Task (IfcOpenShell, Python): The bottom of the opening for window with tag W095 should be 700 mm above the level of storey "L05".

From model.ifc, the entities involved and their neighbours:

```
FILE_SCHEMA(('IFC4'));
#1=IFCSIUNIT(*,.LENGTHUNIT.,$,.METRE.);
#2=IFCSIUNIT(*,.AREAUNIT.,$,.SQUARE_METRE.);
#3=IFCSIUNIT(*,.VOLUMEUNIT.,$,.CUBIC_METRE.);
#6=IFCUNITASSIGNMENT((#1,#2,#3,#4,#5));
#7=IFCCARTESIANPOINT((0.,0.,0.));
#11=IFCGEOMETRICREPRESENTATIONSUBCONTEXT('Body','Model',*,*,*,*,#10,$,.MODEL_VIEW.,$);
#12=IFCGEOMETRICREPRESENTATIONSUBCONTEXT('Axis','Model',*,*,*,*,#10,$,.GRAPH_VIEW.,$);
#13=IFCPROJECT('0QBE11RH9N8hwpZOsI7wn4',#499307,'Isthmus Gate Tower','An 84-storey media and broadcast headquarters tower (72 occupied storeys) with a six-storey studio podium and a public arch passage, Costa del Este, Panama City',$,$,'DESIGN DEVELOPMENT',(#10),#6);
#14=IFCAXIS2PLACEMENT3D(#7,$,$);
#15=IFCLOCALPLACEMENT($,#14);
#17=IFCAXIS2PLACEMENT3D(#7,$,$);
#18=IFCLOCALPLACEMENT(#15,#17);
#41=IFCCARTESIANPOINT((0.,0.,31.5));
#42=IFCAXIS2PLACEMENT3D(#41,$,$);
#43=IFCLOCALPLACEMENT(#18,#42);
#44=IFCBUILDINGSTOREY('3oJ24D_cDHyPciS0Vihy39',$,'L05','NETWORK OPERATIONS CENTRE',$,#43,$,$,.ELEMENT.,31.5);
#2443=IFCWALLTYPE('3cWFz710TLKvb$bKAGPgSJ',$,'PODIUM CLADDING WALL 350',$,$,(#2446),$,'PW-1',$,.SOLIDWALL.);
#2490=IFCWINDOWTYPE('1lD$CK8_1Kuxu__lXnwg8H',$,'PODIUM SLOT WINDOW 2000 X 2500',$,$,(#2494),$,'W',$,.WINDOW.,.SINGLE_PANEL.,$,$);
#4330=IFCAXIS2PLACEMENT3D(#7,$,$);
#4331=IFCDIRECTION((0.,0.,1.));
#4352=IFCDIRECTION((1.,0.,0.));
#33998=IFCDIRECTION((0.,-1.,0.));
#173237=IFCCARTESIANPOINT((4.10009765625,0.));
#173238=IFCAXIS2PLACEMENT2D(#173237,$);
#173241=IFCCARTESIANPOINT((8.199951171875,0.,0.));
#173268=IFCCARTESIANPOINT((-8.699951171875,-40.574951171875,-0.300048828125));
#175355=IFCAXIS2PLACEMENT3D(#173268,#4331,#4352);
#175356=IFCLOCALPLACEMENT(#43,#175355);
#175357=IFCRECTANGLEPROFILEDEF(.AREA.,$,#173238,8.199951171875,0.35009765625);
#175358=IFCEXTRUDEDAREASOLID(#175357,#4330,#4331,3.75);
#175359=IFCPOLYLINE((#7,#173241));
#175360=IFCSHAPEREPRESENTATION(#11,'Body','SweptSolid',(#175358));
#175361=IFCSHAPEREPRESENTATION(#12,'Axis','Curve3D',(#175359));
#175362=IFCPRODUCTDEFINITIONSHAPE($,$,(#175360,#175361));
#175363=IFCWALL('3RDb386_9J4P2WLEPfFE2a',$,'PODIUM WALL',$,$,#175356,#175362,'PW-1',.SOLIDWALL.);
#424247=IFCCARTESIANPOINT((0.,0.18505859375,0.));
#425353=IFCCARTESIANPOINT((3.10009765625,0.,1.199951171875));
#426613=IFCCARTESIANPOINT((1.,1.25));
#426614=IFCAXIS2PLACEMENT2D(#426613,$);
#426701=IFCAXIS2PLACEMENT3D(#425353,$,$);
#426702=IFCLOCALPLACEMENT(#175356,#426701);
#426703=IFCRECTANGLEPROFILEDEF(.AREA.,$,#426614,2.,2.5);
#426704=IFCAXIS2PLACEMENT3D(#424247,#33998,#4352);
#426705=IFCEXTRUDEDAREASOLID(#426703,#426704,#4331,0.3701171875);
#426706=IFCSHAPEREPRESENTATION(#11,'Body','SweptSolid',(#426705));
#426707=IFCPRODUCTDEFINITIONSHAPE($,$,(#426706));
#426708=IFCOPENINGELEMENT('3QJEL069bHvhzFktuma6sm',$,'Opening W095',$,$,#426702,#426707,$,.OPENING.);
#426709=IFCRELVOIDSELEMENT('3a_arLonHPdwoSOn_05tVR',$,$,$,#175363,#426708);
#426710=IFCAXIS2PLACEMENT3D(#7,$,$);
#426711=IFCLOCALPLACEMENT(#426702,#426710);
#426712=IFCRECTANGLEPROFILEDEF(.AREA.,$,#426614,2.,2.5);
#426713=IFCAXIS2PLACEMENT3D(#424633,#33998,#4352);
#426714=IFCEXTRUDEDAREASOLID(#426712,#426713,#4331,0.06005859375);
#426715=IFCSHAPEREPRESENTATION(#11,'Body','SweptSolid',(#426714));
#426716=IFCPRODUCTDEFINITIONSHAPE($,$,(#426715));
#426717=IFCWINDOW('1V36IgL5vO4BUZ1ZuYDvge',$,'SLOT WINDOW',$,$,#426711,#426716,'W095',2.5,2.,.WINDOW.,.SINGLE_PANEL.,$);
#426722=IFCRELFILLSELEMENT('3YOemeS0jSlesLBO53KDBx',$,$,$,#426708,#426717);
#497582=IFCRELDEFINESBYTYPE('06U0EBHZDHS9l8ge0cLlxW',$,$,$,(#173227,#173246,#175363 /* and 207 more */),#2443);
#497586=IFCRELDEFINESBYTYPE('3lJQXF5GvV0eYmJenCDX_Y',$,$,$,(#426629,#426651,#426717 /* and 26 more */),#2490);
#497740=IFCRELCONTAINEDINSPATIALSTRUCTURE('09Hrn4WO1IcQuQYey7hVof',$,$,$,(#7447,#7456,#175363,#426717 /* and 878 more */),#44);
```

```python
import numpy as np
import ifcopenshell
import ifcopenshell.api.geometry
import ifcopenshell.geom
import ifcopenshell.util.element
import ifcopenshell.util.placement
import ifcopenshell.util.shape
import ifcopenshell.util.unit

model = ifcopenshell.open("model.ifc")
unit_scale = ifcopenshell.util.unit.calculate_unit_scale(model)

window = model.by_guid("1V36IgL5vO4BUZ1ZuYDvge")
opening = window.FillsVoids[0].RelatingOpeningElement
storey = ifcopenshell.util.element.get_container(window, ifc_class="IfcBuildingStorey")
level = ifcopenshell.util.placement.get_local_placement(storey.ObjectPlacement)[2, 3]

# The opening's origin need not be at the sill, so measure its lowest point.
shape = ifcopenshell.geom.create_shape(ifcopenshell.geom.settings(), opening)
bottom = ifcopenshell.util.shape.get_shape_bottom_elevation(shape, shape.geometry) / unit_scale
dz = level + 0.7 / unit_scale - bottom

shift = np.array([0.0, 0.0, dz])
# The window is placed relative to its opening, so it follows when the opening moves.
matrix = ifcopenshell.util.placement.get_local_placement(opening.ObjectPlacement)
matrix[:3, 3] += shift
ifcopenshell.api.geometry.edit_object_placement(
    model, product=opening, matrix=matrix, is_si=False, should_transform_children=True
)

print(f"moved by {dz * unit_scale:+.3f} m")

model.write("model_edited.ifc")
```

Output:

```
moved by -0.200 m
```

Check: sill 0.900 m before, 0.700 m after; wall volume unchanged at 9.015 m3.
